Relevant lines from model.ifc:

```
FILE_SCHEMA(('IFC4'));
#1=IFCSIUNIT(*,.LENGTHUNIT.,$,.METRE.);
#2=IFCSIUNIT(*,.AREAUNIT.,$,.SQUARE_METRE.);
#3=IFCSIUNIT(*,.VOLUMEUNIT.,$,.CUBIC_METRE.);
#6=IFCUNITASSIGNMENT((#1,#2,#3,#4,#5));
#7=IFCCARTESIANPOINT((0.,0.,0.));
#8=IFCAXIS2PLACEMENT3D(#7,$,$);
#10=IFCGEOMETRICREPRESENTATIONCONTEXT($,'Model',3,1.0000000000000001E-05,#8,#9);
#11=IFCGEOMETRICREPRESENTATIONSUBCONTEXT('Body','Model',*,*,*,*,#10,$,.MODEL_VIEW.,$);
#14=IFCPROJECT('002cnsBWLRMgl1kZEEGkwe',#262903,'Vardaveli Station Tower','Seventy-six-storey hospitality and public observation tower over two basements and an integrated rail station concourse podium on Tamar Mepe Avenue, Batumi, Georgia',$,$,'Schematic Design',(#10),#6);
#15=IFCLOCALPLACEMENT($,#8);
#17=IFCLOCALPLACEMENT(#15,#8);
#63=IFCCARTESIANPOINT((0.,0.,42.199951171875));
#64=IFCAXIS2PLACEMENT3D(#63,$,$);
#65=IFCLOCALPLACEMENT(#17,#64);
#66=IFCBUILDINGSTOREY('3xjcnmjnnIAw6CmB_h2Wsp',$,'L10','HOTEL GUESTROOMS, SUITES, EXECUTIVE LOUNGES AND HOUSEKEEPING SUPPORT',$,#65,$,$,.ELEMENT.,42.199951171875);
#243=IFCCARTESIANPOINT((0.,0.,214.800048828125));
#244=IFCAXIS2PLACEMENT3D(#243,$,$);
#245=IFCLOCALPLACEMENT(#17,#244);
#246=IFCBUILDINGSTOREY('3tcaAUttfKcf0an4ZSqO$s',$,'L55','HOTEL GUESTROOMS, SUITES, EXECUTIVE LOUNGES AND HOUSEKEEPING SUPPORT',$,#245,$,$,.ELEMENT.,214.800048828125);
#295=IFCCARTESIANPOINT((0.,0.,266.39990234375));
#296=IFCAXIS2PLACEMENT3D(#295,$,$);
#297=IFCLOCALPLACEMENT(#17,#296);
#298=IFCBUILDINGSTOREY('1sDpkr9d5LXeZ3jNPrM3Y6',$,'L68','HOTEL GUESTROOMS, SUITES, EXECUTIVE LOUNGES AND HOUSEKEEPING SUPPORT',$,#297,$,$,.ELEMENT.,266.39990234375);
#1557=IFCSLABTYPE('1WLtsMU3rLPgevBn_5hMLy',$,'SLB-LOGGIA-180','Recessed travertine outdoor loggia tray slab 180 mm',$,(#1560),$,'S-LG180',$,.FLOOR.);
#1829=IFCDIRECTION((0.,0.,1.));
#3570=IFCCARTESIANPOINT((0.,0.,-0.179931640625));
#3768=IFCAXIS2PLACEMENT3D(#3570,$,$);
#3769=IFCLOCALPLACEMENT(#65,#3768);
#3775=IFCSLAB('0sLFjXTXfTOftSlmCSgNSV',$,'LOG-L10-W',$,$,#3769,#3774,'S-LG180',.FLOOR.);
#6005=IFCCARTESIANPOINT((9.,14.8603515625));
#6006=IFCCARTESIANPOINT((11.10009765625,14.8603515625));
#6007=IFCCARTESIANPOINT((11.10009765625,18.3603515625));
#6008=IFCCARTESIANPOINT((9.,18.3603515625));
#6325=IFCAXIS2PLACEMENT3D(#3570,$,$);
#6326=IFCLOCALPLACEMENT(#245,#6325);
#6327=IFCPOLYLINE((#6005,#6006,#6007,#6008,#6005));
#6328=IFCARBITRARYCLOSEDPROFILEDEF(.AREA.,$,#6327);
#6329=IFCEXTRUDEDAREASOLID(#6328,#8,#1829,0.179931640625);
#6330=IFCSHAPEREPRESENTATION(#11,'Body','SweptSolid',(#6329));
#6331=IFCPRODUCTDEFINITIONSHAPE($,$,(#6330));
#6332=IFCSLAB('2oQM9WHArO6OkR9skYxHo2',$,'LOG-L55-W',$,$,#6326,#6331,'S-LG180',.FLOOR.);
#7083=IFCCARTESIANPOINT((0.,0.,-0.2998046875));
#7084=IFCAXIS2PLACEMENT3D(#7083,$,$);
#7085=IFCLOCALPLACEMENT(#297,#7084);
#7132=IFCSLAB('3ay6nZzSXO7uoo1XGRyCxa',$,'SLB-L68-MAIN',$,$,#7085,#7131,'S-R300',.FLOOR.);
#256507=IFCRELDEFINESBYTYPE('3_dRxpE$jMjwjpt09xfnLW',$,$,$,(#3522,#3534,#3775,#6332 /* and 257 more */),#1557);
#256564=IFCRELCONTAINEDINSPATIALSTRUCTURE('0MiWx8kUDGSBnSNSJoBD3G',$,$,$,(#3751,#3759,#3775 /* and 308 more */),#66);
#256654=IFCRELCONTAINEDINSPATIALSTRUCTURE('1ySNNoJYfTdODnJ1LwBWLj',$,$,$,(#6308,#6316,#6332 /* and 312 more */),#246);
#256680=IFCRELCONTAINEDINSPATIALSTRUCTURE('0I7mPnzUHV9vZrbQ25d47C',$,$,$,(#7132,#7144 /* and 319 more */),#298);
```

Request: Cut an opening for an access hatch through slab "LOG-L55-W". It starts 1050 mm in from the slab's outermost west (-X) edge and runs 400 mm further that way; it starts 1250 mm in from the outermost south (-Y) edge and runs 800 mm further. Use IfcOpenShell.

```python
import numpy as np
import ifcopenshell
import ifcopenshell.api.feature
import ifcopenshell.api.geometry
import ifcopenshell.api.root
import ifcopenshell.geom
import ifcopenshell.util.placement
import ifcopenshell.util.representation
import ifcopenshell.util.shape
import ifcopenshell.util.unit

model = ifcopenshell.open("model.ifc")
unit_scale = ifcopenshell.util.unit.calculate_unit_scale(model)
settings = ifcopenshell.geom.settings()


def volume(element):
    """Net volume in cubic metres, openings subtracted."""
    shape = ifcopenshell.geom.create_shape(settings, element)
    return ifcopenshell.util.shape.get_volume(shape.geometry)


slab = model.by_guid("2oQM9WHArO6OkR9skYxHo2")
before = volume(slab)

# Extent in the slab's own axes, in metres. The edges named are its -X and -Y sides.
slab_shape = ifcopenshell.geom.create_shape(settings, slab)
vertices = ifcopenshell.util.shape.get_vertices(slab_shape.geometry)
x_min, y_min, bottom = vertices.min(axis=0)
top = vertices[:, 2].max()

opening = ifcopenshell.api.root.create_entity(model, ifc_class="IfcOpeningElement", name="Access hatch opening", predefined_type="OPENING")
context = ifcopenshell.util.representation.get_context(model, "Model", "Body", "MODEL_VIEW")
width, depth = 0.4, 0.8
outline = [(0.0, 0.0), (width, 0.0), (width, depth), (0.0, depth), (0.0, 0.0)]
# Overshoot both faces by 50 mm so the cut is clean.
shape = ifcopenshell.api.geometry.add_slab_representation(
    model, context=context, depth=top - bottom + 0.1, polyline=outline
)
ifcopenshell.api.geometry.assign_representation(model, product=opening, representation=shape)

matrix = ifcopenshell.util.placement.get_local_placement(slab.ObjectPlacement)
matrix[:, 3] = matrix @ np.append(np.array([x_min + 1.05, y_min + 1.25, bottom - 0.05]) / unit_scale, 1.0)
ifcopenshell.api.geometry.edit_object_placement(model, product=opening, matrix=matrix, is_si=False)
ifcopenshell.api.feature.add_feature(model, feature=opening, element=slab)

after = volume(slab)

print(f"slab volume {before:.3f} -> {after:.3f} m3")

model.write("model_updated.ifc")
```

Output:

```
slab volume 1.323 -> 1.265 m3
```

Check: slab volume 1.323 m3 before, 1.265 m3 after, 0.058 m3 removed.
